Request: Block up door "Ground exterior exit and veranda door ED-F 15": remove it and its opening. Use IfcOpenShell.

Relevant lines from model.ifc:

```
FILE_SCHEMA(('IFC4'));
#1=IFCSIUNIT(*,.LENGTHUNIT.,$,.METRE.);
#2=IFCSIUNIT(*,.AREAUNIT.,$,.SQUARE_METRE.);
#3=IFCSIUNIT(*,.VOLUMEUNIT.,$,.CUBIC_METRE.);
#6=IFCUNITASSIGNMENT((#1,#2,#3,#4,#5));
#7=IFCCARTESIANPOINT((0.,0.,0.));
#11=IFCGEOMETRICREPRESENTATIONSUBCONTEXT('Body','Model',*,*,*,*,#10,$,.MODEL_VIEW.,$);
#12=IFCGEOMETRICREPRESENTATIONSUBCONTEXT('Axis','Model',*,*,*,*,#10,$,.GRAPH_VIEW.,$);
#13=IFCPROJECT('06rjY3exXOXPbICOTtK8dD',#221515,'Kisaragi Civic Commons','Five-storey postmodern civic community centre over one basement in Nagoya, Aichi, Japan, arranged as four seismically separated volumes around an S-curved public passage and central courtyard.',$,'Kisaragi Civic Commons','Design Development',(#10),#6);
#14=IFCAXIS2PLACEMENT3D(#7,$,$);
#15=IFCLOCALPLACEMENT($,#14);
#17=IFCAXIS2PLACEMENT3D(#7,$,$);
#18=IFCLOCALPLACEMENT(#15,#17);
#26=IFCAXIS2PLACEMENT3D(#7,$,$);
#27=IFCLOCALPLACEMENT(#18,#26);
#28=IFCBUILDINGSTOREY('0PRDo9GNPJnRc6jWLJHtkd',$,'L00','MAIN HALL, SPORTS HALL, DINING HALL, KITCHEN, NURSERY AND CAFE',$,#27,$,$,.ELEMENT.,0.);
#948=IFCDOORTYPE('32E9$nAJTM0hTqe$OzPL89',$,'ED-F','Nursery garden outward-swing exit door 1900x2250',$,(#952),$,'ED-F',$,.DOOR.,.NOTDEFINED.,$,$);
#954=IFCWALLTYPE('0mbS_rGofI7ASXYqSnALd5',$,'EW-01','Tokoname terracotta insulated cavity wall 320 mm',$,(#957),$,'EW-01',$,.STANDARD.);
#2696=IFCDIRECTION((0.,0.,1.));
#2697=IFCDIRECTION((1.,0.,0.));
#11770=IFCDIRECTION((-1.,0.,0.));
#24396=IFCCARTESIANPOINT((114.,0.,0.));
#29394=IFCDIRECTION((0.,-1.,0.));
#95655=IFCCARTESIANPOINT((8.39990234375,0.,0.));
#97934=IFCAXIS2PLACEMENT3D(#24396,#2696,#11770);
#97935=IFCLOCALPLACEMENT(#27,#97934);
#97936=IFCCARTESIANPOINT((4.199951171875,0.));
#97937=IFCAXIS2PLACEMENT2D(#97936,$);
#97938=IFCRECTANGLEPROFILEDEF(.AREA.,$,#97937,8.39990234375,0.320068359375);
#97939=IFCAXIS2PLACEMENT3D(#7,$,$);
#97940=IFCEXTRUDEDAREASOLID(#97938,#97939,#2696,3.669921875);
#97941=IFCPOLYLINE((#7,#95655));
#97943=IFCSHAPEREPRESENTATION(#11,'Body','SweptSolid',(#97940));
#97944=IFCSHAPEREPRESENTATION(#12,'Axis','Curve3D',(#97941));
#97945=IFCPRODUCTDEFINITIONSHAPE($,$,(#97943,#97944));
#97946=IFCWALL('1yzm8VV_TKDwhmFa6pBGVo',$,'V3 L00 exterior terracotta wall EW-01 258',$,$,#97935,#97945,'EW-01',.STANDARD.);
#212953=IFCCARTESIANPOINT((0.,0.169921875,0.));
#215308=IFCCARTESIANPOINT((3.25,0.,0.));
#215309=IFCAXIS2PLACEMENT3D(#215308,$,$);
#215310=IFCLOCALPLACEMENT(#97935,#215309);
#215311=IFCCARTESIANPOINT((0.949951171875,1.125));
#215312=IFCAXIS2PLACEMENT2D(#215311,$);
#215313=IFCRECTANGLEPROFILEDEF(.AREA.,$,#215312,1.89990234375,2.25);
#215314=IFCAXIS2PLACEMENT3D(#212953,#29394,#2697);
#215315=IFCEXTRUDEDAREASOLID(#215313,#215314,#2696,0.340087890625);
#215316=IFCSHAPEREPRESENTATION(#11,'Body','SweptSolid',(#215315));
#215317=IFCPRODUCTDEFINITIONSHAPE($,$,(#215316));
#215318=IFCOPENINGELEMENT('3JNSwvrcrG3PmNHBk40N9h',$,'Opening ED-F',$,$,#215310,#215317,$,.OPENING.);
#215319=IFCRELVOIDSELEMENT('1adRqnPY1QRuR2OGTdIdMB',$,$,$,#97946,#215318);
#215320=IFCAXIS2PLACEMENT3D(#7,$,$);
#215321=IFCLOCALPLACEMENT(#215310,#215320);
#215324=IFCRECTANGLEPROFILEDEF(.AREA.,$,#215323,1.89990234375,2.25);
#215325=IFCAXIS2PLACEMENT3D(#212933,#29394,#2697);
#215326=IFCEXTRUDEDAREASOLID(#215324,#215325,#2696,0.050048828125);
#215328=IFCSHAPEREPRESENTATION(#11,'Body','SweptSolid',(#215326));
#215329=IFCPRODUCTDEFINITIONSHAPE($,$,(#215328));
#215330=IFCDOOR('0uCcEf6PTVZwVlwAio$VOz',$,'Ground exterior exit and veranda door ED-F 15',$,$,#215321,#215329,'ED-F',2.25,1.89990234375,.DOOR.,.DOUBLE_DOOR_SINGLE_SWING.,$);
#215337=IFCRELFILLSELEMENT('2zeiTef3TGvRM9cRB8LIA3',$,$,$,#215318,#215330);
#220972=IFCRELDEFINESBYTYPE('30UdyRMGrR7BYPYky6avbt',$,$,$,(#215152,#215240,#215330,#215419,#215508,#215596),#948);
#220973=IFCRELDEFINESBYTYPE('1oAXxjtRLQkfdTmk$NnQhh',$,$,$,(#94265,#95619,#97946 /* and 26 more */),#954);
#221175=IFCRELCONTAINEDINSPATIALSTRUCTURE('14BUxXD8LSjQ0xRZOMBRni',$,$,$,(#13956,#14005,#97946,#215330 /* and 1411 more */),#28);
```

```python
import ifcopenshell
import ifcopenshell.api.feature
import ifcopenshell.api.root
import ifcopenshell.geom
import ifcopenshell.util.shape

model = ifcopenshell.open("model.ifc")
settings = ifcopenshell.geom.settings()


def volume(element):
    """Net volume in cubic metres, openings subtracted."""
    shape = ifcopenshell.geom.create_shape(settings, element)
    return ifcopenshell.util.shape.get_volume(shape.geometry)


door = model.by_guid("0uCcEf6PTVZwVlwAio$VOz")
opening = door.FillsVoids[0].RelatingOpeningElement
wall = opening.VoidsElements[0].RelatingBuildingElement
before = volume(wall)

ifcopenshell.api.root.remove_product(model, product=door)
ifcopenshell.api.feature.remove_feature(model, feature=opening)

after = volume(wall)

print(f"wall volume {before:.3f} -> {after:.3f} m3")

model.write("model_edited.ifc")
```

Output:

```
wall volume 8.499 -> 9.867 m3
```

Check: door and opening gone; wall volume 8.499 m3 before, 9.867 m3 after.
